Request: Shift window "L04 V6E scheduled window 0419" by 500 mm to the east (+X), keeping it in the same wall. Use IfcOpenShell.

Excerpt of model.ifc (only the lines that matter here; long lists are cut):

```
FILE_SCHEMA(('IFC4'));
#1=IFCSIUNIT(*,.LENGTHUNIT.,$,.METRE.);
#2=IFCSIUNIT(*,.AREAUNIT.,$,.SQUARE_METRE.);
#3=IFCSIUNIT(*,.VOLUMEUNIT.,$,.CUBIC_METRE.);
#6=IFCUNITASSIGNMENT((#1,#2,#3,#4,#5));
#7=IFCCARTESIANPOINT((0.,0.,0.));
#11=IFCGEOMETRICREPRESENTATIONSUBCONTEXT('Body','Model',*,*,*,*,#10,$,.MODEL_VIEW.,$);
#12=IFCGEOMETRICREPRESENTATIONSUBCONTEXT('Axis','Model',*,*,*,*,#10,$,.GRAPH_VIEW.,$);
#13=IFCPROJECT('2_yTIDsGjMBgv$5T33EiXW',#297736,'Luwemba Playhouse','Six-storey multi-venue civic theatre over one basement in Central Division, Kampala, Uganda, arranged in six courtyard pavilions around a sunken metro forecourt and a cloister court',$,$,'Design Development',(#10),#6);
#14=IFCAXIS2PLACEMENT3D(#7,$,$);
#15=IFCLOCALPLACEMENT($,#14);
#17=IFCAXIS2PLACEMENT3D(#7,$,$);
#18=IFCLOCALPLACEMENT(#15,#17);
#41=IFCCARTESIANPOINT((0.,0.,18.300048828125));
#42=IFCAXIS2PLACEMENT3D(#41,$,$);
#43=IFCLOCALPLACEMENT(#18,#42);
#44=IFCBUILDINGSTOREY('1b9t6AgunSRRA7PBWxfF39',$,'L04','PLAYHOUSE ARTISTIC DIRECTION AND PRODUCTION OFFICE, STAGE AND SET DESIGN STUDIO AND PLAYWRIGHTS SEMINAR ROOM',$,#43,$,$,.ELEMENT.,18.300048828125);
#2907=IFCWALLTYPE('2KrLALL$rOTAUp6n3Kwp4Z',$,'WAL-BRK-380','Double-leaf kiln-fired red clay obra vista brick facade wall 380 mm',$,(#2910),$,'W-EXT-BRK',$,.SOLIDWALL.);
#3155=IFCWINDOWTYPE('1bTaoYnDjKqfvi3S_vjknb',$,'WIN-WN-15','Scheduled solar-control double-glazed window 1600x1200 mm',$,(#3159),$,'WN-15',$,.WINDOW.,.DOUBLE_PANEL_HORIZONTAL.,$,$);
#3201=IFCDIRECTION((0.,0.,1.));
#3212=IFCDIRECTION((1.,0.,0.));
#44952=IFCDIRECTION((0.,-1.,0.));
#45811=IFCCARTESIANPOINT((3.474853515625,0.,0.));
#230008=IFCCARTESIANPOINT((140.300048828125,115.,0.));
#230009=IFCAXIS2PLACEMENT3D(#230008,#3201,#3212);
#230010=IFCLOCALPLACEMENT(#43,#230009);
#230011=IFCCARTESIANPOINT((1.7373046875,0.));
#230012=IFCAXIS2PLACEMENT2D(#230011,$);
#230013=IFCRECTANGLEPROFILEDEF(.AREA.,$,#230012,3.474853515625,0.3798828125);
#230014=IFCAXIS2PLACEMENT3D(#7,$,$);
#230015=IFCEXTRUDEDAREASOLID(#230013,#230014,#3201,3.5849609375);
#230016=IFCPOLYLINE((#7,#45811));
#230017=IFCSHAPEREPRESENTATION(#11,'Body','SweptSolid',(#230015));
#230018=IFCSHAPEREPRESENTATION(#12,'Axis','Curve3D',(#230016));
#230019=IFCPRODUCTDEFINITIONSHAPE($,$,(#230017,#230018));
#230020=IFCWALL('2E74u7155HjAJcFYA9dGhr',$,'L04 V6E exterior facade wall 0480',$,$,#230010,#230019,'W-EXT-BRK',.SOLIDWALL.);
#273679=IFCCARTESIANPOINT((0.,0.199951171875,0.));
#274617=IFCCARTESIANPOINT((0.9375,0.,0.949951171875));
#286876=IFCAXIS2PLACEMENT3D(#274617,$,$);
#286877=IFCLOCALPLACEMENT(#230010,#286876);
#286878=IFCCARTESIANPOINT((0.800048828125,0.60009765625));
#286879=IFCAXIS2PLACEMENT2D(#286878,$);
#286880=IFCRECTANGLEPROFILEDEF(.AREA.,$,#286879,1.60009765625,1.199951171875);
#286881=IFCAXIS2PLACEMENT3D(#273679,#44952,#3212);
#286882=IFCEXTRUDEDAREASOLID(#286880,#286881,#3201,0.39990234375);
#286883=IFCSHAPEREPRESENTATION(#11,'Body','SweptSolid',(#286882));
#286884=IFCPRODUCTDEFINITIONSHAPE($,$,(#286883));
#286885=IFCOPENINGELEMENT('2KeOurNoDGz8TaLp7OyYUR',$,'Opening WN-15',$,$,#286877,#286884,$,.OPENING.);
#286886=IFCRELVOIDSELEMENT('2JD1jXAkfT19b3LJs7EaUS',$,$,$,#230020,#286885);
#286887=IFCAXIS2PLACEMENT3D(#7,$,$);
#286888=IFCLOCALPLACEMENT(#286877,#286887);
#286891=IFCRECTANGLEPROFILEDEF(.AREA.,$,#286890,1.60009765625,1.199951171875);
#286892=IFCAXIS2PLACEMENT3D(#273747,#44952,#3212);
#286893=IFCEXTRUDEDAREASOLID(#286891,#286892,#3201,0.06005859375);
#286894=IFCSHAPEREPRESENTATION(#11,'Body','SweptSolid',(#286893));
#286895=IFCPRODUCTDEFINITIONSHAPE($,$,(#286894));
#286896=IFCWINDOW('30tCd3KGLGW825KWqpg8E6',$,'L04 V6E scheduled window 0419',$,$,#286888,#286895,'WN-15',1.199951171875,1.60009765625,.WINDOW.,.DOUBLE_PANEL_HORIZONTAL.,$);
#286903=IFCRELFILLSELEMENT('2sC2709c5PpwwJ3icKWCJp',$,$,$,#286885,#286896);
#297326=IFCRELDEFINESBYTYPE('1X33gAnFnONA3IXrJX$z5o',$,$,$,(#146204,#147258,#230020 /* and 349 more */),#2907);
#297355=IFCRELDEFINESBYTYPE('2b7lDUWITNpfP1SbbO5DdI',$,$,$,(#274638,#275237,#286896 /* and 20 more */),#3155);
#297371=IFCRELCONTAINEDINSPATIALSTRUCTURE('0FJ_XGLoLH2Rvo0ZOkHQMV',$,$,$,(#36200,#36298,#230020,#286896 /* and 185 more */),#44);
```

```python
import ifcopenshell
import ifcopenshell.api.geometry
import ifcopenshell.util.placement
import ifcopenshell.util.unit

model = ifcopenshell.open("model.ifc")
unit_scale = ifcopenshell.util.unit.calculate_unit_scale(model)

window = model.by_guid("30tCd3KGLGW825KWqpg8E6")
opening = window.FillsVoids[0].RelatingOpeningElement
wall = opening.VoidsElements[0].RelatingBuildingElement

wall_matrix = ifcopenshell.util.placement.get_local_placement(wall.ObjectPlacement)
shift = wall_matrix[:3, 0] * 0.5 / unit_scale
before = ifcopenshell.util.placement.get_local_placement(window.ObjectPlacement)[:3, 3].copy()

# The window is placed relative to its opening, so it follows when the opening moves.
matrix = ifcopenshell.util.placement.get_local_placement(opening.ObjectPlacement)
matrix[:3, 3] += shift
ifcopenshell.api.geometry.edit_object_placement(
    model, product=opening, matrix=matrix, is_si=False, should_transform_children=True
)

after = ifcopenshell.util.placement.get_local_placement(window.ObjectPlacement)[:3, 3]
print("window moved by", (after - before).round(3) + 0.0)

model.write("model_updated.ifc")
```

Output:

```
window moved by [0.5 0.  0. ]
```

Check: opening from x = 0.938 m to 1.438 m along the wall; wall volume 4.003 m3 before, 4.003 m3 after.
